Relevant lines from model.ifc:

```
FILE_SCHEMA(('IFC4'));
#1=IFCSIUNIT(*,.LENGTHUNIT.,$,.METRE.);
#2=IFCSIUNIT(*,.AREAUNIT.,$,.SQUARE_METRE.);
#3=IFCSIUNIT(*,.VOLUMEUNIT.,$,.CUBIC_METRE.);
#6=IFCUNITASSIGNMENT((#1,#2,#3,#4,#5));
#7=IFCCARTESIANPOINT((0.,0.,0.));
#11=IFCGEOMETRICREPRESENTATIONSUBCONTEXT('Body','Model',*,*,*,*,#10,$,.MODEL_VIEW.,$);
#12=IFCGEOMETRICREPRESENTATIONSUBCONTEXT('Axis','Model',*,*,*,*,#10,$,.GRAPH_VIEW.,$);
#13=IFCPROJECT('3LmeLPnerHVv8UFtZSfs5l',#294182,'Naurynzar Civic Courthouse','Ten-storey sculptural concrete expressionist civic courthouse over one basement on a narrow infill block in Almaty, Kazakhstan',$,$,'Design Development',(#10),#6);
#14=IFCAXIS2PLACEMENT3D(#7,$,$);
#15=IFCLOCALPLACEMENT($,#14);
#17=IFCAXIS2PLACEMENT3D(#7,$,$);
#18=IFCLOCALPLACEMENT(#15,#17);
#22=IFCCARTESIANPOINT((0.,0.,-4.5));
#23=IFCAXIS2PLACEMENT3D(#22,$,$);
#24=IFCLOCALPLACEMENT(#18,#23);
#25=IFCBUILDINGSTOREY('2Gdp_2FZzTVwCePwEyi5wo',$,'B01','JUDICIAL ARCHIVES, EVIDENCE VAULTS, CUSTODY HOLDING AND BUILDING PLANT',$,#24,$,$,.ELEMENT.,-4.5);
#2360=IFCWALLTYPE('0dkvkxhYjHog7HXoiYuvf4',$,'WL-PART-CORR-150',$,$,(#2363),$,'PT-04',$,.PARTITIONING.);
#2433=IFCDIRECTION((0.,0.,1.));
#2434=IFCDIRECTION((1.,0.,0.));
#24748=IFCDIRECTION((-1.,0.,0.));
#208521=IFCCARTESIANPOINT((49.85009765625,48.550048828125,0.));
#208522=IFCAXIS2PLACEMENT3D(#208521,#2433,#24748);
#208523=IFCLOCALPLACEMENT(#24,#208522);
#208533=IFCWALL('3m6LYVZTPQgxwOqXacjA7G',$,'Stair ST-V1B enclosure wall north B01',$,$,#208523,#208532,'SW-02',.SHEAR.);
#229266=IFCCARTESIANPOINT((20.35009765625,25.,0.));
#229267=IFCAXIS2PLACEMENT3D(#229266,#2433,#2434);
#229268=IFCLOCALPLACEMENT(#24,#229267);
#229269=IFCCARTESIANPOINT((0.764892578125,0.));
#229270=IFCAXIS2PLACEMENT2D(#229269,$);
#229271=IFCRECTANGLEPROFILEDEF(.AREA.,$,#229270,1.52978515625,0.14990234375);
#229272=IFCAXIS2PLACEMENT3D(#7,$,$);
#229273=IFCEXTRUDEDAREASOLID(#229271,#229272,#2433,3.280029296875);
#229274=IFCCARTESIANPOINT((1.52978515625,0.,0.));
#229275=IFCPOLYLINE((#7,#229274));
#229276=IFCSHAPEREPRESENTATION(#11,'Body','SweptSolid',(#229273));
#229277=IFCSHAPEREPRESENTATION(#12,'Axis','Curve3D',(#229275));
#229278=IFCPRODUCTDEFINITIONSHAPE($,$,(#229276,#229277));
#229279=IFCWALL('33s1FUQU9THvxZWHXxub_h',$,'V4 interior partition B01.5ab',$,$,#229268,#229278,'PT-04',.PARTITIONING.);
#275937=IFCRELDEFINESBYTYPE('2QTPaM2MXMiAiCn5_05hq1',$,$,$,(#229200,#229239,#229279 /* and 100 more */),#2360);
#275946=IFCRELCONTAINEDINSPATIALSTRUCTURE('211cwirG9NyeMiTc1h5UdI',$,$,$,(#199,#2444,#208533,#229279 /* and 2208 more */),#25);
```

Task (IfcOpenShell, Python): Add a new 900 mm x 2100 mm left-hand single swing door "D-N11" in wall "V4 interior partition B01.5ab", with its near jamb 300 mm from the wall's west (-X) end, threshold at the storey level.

```python
import numpy as np
import ifcopenshell
import ifcopenshell.api.feature
import ifcopenshell.api.geometry
import ifcopenshell.api.root
import ifcopenshell.api.spatial
import ifcopenshell.geom
import ifcopenshell.util.element
import ifcopenshell.util.placement
import ifcopenshell.util.representation
import ifcopenshell.util.shape
import ifcopenshell.util.unit

model = ifcopenshell.open("model.ifc")
unit_scale = ifcopenshell.util.unit.calculate_unit_scale(model)
settings = ifcopenshell.geom.settings()


def volume(element):
    """Net volume in cubic metres, openings subtracted."""
    shape = ifcopenshell.geom.create_shape(settings, element)
    return ifcopenshell.util.shape.get_volume(shape.geometry)


wall = model.by_guid("33s1FUQU9THvxZWHXxub_h")
storey = ifcopenshell.util.element.get_container(wall, ifc_class="IfcBuildingStorey")
context = ifcopenshell.util.representation.get_context(model, "Model", "Body", "MODEL_VIEW")
before = volume(wall)

width, height, from_end, sill = 0.9, 2.1, 0.3, 0.0  # metres

# The wall runs along its own X axis, and the end named is its -X end.
wall_shape = ifcopenshell.geom.create_shape(settings, wall)
x, y, z = ifcopenshell.util.shape.get_vertices(wall_shape.geometry).T
start = x.min() + from_end
face, thickness = float(y.min()), float(y.max() - y.min())
wall_matrix = ifcopenshell.util.placement.get_local_placement(wall.ObjectPlacement)
level = ifcopenshell.util.placement.get_local_placement(storey.ObjectPlacement)[2, 3]


def in_wall(x, y):
    """Placement at x, y metres in the wall's axes, at sill height."""
    matrix = wall_matrix.copy()
    matrix[:, 3] = wall_matrix @ np.array([x / unit_scale, y / unit_scale, 0.0, 1.0])
    matrix[2, 3] = level + sill / unit_scale
    return matrix


# Opening: a box that overshoots both wall faces by 50 mm.
opening = ifcopenshell.api.root.create_entity(model, ifc_class="IfcOpeningElement", predefined_type="OPENING")
box = ifcopenshell.api.geometry.add_wall_representation(
    model, context=context, length=width, height=height, thickness=thickness + 0.1
)
ifcopenshell.api.geometry.assign_representation(model, product=opening, representation=box)
ifcopenshell.api.geometry.edit_object_placement(model, product=opening, matrix=in_wall(start, face - 0.05), is_si=False)
ifcopenshell.api.feature.add_feature(model, feature=opening, element=wall)

door = ifcopenshell.api.root.create_entity(model, ifc_class="IfcDoor", name="D-N11", predefined_type="DOOR")
door.OverallWidth, door.OverallHeight = width / unit_scale, height / unit_scale
door.OperationType = "SINGLE_SWING_LEFT"
body = ifcopenshell.api.geometry.add_door_representation(
    model,
    context=context,
    overall_width=door.OverallWidth,
    overall_height=door.OverallHeight,
    operation_type="SINGLE_SWING_LEFT",
    lining_properties={"LiningDepth": thickness / unit_scale, "ThresholdDepth": thickness / unit_scale},
)
ifcopenshell.api.geometry.assign_representation(model, product=door, representation=body)
ifcopenshell.api.spatial.assign_container(model, products=[door], relating_structure=storey)
ifcopenshell.api.feature.add_filling(model, opening=opening, element=door)

# The lining spans the wall, so the door starts at the wall face.
ifcopenshell.api.geometry.edit_object_placement(model, product=door, matrix=in_wall(start, face), is_si=False)

after = volume(wall)

print(f"wall volume {before:.3f} -> {after:.3f} m3")

model.write("model_edited.ifc")
```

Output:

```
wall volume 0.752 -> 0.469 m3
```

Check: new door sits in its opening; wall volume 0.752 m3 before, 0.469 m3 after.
